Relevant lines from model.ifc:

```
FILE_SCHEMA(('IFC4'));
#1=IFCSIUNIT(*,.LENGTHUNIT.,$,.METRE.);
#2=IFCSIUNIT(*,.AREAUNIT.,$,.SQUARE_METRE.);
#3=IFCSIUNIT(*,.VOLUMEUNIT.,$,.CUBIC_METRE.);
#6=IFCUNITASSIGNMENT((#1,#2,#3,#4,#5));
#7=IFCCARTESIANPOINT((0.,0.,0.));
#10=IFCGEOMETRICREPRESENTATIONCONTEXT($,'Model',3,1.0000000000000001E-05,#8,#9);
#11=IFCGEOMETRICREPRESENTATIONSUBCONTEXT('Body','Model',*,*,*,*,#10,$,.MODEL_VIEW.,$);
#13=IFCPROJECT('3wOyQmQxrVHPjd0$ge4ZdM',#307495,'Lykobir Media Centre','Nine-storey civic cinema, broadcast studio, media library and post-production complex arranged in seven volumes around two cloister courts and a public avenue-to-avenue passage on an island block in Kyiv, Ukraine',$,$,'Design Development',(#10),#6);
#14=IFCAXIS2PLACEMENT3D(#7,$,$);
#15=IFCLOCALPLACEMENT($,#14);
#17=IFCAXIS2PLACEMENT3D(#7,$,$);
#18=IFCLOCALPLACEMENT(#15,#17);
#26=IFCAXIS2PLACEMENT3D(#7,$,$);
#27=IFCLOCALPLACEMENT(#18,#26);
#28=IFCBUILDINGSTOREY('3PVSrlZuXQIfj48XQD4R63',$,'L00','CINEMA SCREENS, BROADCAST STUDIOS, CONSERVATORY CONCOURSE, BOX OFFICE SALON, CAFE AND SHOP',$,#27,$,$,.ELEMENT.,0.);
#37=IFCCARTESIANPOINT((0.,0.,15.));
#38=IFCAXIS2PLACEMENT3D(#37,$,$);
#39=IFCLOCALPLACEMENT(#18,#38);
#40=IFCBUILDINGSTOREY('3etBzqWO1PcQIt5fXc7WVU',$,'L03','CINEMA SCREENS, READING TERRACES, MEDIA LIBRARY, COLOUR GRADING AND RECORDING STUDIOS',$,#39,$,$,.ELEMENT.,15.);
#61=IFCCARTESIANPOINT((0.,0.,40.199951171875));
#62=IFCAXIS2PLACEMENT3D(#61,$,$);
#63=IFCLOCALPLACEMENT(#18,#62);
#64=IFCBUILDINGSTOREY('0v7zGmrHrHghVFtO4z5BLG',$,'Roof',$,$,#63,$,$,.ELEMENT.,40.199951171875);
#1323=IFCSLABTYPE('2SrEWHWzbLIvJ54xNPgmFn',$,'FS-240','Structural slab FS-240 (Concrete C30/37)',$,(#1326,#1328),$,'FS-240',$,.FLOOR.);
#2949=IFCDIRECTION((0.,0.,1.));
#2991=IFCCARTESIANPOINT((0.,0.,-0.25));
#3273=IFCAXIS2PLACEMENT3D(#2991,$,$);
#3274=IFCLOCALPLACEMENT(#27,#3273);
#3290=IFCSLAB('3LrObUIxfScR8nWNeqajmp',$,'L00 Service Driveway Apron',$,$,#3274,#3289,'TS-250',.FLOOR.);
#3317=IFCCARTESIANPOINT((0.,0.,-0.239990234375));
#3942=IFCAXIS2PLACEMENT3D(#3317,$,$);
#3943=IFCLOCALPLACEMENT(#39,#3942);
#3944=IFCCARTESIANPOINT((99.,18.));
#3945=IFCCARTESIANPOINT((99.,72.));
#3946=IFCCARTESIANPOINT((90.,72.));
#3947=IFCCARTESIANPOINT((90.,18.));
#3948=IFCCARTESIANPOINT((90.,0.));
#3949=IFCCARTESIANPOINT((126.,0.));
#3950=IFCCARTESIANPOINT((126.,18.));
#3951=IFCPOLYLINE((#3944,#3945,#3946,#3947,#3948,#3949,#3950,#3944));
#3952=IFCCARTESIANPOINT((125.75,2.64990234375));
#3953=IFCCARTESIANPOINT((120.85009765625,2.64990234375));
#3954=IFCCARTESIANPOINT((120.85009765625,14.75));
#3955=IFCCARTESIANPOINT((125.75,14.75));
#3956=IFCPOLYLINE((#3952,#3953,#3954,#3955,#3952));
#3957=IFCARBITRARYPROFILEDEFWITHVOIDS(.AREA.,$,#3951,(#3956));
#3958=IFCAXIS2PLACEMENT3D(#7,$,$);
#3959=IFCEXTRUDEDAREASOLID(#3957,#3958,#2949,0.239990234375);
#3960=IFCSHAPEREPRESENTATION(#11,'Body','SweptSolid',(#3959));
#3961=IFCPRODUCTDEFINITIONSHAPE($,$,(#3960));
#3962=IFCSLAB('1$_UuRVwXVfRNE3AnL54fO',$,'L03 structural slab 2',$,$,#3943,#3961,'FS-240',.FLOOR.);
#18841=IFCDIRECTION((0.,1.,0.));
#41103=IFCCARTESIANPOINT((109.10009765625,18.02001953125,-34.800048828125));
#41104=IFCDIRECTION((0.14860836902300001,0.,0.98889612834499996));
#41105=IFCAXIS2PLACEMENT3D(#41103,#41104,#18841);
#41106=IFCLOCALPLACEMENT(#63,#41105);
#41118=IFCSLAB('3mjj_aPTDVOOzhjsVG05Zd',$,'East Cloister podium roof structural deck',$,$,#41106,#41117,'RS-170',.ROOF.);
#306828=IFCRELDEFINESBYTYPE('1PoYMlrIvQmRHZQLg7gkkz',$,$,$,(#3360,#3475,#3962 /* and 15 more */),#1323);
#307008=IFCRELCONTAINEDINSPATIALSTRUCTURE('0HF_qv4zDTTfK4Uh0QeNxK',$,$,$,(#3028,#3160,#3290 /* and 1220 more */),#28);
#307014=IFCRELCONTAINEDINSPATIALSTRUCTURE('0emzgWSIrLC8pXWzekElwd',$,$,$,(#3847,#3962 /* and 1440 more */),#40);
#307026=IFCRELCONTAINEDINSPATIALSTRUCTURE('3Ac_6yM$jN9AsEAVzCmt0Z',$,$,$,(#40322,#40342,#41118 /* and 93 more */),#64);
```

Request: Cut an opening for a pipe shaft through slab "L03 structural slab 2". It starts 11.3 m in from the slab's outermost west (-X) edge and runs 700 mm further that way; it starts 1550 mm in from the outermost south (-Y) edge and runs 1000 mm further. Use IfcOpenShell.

```python
import numpy as np
import ifcopenshell
import ifcopenshell.api.feature
import ifcopenshell.api.geometry
import ifcopenshell.api.root
import ifcopenshell.geom
import ifcopenshell.util.placement
import ifcopenshell.util.representation
import ifcopenshell.util.shape
import ifcopenshell.util.unit

model = ifcopenshell.open("model.ifc")
unit_scale = ifcopenshell.util.unit.calculate_unit_scale(model)
settings = ifcopenshell.geom.settings()


def volume(element):
    """Net volume in cubic metres, openings subtracted."""
    shape = ifcopenshell.geom.create_shape(settings, element)
    return ifcopenshell.util.shape.get_volume(shape.geometry)


slab = model.by_guid("1$_UuRVwXVfRNE3AnL54fO")
before = volume(slab)

# Extent in the slab's own axes, in metres. The edges named are its -X and -Y sides.
slab_shape = ifcopenshell.geom.create_shape(settings, slab)
vertices = ifcopenshell.util.shape.get_vertices(slab_shape.geometry)
x_min, y_min, bottom = vertices.min(axis=0)
top = vertices[:, 2].max()

opening = ifcopenshell.api.root.create_entity(model, ifc_class="IfcOpeningElement", name="Pipe shaft opening", predefined_type="OPENING")
context = ifcopenshell.util.representation.get_context(model, "Model", "Body", "MODEL_VIEW")
width, depth = 0.7, 1
outline = [(0.0, 0.0), (width, 0.0), (width, depth), (0.0, depth), (0.0, 0.0)]
# Overshoot both faces by 50 mm so the cut is clean.
shape = ifcopenshell.api.geometry.add_slab_representation(
    model, context=context, depth=top - bottom + 0.1, polyline=outline
)
ifcopenshell.api.geometry.assign_representation(model, product=opening, representation=shape)

matrix = ifcopenshell.util.placement.get_local_placement(slab.ObjectPlacement)
matrix[:, 3] = matrix @ np.append(np.array([x_min + 11.3, y_min + 1.55, bottom - 0.05]) / unit_scale, 1.0)
ifcopenshell.api.geometry.edit_object_placement(model, product=opening, matrix=matrix, is_si=False)
ifcopenshell.api.feature.add_feature(model, feature=opening, element=slab)

after = volume(slab)

print(f"slab volume {before:.3f} -> {after:.3f} m3")

model.write("model-out.ifc")
```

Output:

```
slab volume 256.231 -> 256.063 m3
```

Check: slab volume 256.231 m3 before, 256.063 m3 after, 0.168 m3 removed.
